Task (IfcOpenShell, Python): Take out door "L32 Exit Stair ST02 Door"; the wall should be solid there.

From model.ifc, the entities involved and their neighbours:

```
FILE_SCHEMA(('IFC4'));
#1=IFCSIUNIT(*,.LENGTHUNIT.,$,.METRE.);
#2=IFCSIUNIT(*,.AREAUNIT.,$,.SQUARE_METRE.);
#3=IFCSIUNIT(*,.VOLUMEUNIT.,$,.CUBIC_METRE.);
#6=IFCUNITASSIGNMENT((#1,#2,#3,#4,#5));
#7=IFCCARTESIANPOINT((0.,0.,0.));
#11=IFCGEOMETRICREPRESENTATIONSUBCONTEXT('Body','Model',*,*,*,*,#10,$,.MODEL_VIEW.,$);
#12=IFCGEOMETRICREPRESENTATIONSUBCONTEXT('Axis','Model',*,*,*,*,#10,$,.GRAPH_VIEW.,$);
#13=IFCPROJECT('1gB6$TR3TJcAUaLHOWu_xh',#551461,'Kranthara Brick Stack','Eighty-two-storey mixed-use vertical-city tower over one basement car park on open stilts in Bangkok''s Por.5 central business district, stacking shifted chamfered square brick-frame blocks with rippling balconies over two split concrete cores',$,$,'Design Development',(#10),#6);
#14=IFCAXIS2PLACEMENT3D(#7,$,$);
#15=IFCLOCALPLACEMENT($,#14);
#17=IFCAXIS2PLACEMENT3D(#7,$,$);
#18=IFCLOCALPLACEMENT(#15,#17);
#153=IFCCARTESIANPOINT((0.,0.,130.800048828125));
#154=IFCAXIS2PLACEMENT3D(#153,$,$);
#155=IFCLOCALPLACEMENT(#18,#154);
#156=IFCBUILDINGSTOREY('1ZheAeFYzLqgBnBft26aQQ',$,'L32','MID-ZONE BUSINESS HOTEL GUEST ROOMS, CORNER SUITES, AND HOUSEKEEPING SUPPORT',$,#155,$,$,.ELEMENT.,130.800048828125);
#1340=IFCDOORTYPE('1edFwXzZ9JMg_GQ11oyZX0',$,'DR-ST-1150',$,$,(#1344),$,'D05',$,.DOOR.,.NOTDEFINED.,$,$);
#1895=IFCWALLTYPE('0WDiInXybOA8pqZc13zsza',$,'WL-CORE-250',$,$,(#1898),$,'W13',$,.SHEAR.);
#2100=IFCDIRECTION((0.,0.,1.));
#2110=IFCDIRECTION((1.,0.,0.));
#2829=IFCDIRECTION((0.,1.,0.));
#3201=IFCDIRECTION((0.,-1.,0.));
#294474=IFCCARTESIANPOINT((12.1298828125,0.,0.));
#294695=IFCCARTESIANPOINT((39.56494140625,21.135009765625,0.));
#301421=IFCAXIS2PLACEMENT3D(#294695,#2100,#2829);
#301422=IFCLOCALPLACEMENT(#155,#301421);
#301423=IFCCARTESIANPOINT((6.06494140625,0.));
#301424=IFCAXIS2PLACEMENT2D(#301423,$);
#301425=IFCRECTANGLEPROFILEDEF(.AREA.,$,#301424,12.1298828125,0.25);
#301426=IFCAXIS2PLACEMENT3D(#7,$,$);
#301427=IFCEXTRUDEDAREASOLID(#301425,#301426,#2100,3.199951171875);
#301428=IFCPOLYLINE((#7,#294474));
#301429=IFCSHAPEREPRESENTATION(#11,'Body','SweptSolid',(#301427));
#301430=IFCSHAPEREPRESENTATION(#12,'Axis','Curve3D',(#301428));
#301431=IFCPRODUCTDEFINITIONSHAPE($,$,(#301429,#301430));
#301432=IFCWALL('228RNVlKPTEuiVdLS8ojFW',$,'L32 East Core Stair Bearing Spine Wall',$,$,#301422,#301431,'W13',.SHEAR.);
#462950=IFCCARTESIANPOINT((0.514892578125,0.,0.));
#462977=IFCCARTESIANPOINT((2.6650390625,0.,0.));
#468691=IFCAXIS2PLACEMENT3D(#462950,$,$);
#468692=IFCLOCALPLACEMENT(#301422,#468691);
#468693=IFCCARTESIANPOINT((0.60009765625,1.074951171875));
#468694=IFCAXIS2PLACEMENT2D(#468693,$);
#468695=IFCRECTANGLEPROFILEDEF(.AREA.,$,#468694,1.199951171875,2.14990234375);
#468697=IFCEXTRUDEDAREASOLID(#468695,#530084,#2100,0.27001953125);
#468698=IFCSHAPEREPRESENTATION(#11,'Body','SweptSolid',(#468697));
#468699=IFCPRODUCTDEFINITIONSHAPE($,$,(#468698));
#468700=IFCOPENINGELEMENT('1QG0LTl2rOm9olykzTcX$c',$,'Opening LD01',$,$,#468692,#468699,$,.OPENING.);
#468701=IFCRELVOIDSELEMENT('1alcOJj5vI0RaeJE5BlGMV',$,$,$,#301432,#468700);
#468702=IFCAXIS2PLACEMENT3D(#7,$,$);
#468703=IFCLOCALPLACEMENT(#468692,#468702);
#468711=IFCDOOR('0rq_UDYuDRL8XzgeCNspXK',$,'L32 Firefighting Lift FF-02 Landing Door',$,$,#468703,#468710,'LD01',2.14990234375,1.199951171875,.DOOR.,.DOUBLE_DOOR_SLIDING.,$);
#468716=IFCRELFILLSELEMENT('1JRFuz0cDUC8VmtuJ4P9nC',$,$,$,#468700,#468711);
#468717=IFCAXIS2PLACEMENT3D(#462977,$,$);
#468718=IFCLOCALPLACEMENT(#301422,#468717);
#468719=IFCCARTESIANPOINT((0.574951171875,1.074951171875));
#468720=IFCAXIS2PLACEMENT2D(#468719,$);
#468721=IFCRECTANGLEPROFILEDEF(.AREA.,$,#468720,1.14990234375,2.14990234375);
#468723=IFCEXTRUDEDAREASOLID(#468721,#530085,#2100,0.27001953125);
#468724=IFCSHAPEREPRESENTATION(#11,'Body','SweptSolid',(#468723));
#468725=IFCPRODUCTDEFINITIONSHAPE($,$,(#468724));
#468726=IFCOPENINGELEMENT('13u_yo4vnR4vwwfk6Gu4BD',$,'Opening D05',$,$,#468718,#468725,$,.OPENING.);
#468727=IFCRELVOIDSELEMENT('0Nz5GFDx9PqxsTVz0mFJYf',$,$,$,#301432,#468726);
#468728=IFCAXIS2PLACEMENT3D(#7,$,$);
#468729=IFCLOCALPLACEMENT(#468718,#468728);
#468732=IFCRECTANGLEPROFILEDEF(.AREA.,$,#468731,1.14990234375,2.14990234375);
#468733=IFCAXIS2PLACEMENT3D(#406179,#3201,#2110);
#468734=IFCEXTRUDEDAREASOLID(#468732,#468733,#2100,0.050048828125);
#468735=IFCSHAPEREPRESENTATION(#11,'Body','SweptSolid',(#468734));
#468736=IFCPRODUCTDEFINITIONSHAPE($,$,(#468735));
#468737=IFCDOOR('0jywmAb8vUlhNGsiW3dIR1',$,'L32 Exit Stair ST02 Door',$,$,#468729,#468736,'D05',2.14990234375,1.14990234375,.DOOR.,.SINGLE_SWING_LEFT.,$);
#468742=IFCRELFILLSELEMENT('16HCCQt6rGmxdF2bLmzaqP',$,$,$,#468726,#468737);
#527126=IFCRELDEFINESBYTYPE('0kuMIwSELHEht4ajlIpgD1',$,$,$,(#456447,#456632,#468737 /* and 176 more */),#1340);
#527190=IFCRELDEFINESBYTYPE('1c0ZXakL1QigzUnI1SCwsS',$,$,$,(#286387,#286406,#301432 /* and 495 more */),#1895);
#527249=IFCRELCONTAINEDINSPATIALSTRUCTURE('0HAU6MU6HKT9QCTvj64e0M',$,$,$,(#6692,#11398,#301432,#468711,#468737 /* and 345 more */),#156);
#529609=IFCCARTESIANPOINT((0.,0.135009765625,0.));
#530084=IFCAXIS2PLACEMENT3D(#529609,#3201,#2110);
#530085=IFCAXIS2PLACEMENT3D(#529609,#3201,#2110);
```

```python
import ifcopenshell
import ifcopenshell.api.feature
import ifcopenshell.api.root
import ifcopenshell.geom
import ifcopenshell.util.shape

model = ifcopenshell.open("model.ifc")
settings = ifcopenshell.geom.settings()


def volume(element):
    """Net volume in cubic metres, openings subtracted."""
    shape = ifcopenshell.geom.create_shape(settings, element)
    return ifcopenshell.util.shape.get_volume(shape.geometry)


door = model.by_id(468737)
opening = door.FillsVoids[0].RelatingOpeningElement
wall = opening.VoidsElements[0].RelatingBuildingElement
before = volume(wall)

ifcopenshell.api.root.remove_product(model, product=door)
ifcopenshell.api.feature.remove_feature(model, feature=opening)

after = volume(wall)

print(f"wall volume {before:.3f} -> {after:.3f} m3")

model.write("model_v2.ifc")
```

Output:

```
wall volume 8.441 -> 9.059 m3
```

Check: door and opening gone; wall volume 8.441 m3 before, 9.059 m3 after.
